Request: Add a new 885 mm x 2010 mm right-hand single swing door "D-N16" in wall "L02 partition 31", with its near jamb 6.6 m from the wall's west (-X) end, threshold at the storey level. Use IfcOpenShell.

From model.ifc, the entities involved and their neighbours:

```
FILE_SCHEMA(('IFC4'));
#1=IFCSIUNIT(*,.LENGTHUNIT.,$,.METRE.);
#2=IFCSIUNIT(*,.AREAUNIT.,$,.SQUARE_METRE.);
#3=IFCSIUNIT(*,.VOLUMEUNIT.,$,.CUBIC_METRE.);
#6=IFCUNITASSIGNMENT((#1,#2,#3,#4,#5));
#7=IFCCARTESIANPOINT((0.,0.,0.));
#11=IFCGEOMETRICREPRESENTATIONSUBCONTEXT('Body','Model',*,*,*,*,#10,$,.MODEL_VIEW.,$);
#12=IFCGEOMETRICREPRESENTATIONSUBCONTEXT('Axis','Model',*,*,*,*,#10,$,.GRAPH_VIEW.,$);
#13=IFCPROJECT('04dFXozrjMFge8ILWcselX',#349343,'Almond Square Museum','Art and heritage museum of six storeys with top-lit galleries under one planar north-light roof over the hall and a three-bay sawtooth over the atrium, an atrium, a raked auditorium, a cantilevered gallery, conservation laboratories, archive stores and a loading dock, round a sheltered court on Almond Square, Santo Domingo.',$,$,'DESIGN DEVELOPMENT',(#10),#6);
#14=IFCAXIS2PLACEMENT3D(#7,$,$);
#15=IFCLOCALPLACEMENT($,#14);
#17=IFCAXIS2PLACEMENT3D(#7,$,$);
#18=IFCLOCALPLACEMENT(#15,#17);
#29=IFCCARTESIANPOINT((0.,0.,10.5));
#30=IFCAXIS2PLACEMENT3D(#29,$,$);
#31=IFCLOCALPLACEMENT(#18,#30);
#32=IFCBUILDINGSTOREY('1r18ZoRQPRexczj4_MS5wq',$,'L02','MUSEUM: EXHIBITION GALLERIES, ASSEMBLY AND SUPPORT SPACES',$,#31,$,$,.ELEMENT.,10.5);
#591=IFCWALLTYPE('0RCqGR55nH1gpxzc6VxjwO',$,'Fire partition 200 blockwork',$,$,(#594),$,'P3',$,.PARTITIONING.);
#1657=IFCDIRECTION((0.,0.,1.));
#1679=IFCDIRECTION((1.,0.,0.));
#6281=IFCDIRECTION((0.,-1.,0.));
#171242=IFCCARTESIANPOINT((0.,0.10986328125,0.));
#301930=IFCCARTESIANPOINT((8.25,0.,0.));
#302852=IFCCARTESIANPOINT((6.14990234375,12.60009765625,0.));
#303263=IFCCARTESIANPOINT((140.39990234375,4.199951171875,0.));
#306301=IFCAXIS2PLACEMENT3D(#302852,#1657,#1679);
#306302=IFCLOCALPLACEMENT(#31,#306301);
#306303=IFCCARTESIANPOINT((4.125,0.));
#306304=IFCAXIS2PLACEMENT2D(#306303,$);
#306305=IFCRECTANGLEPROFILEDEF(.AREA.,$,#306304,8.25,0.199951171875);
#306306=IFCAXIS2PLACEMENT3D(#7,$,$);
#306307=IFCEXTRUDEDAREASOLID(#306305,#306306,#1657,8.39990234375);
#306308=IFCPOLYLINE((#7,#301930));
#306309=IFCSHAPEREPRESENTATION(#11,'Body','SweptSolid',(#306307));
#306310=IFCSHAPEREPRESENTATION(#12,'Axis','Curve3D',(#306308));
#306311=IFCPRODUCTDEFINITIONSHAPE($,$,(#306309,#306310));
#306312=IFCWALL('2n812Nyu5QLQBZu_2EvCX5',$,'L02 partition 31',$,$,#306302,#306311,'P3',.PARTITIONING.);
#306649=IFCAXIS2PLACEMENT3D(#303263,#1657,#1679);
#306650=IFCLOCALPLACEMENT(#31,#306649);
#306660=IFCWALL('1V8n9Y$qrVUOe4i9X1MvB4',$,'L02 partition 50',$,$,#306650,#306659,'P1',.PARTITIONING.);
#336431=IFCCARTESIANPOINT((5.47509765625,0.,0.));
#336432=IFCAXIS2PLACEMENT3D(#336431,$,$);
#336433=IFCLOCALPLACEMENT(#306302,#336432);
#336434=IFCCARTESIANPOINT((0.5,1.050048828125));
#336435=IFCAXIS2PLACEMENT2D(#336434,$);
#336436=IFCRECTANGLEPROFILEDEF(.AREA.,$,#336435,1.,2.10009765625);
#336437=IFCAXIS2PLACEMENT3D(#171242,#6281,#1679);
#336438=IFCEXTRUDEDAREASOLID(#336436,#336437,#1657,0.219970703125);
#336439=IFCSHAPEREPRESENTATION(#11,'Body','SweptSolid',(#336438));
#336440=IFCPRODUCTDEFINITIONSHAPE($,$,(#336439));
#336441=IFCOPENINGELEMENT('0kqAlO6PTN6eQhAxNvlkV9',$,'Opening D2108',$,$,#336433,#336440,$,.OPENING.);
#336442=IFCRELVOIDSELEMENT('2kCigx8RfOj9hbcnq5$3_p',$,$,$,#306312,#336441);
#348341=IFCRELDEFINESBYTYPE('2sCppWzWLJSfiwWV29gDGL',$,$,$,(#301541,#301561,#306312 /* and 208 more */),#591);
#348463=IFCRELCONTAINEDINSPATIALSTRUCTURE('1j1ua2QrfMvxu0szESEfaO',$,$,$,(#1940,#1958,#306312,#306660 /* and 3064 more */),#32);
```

```python
import numpy as np
import ifcopenshell
import ifcopenshell.api.feature
import ifcopenshell.api.geometry
import ifcopenshell.api.root
import ifcopenshell.api.spatial
import ifcopenshell.geom
import ifcopenshell.util.element
import ifcopenshell.util.placement
import ifcopenshell.util.representation
import ifcopenshell.util.shape
import ifcopenshell.util.unit

model = ifcopenshell.open("model.ifc")
unit_scale = ifcopenshell.util.unit.calculate_unit_scale(model)
settings = ifcopenshell.geom.settings()


def volume(element):
    """Net volume in cubic metres, openings subtracted."""
    shape = ifcopenshell.geom.create_shape(settings, element)
    return ifcopenshell.util.shape.get_volume(shape.geometry)


wall = model.by_guid("2n812Nyu5QLQBZu_2EvCX5")
storey = ifcopenshell.util.element.get_container(wall, ifc_class="IfcBuildingStorey")
context = ifcopenshell.util.representation.get_context(model, "Model", "Body", "MODEL_VIEW")
before = volume(wall)

width, height, from_end, sill = 0.885, 2.01, 6.6, 0.0  # metres

# The wall runs along its own X axis, and the end named is its -X end.
wall_shape = ifcopenshell.geom.create_shape(settings, wall)
x, y, z = ifcopenshell.util.shape.get_vertices(wall_shape.geometry).T
start = x.min() + from_end
face, thickness = float(y.min()), float(y.max() - y.min())
wall_matrix = ifcopenshell.util.placement.get_local_placement(wall.ObjectPlacement)
level = ifcopenshell.util.placement.get_local_placement(storey.ObjectPlacement)[2, 3]


def in_wall(x, y):
    """Placement at x, y metres in the wall's axes, at sill height."""
    matrix = wall_matrix.copy()
    matrix[:, 3] = wall_matrix @ np.array([x / unit_scale, y / unit_scale, 0.0, 1.0])
    matrix[2, 3] = level + sill / unit_scale
    return matrix


# Opening: a box that overshoots both wall faces by 50 mm.
opening = ifcopenshell.api.root.create_entity(model, ifc_class="IfcOpeningElement", predefined_type="OPENING")
box = ifcopenshell.api.geometry.add_wall_representation(
    model, context=context, length=width, height=height, thickness=thickness + 0.1
)
ifcopenshell.api.geometry.assign_representation(model, product=opening, representation=box)
ifcopenshell.api.geometry.edit_object_placement(model, product=opening, matrix=in_wall(start, face - 0.05), is_si=False)
ifcopenshell.api.feature.add_feature(model, feature=opening, element=wall)

door = ifcopenshell.api.root.create_entity(model, ifc_class="IfcDoor", name="D-N16", predefined_type="DOOR")
door.OverallWidth, door.OverallHeight = width / unit_scale, height / unit_scale
door.OperationType = "SINGLE_SWING_RIGHT"
body = ifcopenshell.api.geometry.add_door_representation(
    model,
    context=context,
    overall_width=door.OverallWidth,
    overall_height=door.OverallHeight,
    operation_type="SINGLE_SWING_RIGHT",
    lining_properties={"LiningDepth": thickness / unit_scale, "ThresholdDepth": thickness / unit_scale},
)
ifcopenshell.api.geometry.assign_representation(model, product=door, representation=body)
ifcopenshell.api.spatial.assign_container(model, products=[door], relating_structure=storey)
ifcopenshell.api.feature.add_filling(model, opening=opening, element=door)

# The lining spans the wall, so the door starts at the wall face.
ifcopenshell.api.geometry.edit_object_placement(model, product=door, matrix=in_wall(start, face), is_si=False)

after = volume(wall)

print(f"wall volume {before:.3f} -> {after:.3f} m3")

model.write("model_edited.ifc")
```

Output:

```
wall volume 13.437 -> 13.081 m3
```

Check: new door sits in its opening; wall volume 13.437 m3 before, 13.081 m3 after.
